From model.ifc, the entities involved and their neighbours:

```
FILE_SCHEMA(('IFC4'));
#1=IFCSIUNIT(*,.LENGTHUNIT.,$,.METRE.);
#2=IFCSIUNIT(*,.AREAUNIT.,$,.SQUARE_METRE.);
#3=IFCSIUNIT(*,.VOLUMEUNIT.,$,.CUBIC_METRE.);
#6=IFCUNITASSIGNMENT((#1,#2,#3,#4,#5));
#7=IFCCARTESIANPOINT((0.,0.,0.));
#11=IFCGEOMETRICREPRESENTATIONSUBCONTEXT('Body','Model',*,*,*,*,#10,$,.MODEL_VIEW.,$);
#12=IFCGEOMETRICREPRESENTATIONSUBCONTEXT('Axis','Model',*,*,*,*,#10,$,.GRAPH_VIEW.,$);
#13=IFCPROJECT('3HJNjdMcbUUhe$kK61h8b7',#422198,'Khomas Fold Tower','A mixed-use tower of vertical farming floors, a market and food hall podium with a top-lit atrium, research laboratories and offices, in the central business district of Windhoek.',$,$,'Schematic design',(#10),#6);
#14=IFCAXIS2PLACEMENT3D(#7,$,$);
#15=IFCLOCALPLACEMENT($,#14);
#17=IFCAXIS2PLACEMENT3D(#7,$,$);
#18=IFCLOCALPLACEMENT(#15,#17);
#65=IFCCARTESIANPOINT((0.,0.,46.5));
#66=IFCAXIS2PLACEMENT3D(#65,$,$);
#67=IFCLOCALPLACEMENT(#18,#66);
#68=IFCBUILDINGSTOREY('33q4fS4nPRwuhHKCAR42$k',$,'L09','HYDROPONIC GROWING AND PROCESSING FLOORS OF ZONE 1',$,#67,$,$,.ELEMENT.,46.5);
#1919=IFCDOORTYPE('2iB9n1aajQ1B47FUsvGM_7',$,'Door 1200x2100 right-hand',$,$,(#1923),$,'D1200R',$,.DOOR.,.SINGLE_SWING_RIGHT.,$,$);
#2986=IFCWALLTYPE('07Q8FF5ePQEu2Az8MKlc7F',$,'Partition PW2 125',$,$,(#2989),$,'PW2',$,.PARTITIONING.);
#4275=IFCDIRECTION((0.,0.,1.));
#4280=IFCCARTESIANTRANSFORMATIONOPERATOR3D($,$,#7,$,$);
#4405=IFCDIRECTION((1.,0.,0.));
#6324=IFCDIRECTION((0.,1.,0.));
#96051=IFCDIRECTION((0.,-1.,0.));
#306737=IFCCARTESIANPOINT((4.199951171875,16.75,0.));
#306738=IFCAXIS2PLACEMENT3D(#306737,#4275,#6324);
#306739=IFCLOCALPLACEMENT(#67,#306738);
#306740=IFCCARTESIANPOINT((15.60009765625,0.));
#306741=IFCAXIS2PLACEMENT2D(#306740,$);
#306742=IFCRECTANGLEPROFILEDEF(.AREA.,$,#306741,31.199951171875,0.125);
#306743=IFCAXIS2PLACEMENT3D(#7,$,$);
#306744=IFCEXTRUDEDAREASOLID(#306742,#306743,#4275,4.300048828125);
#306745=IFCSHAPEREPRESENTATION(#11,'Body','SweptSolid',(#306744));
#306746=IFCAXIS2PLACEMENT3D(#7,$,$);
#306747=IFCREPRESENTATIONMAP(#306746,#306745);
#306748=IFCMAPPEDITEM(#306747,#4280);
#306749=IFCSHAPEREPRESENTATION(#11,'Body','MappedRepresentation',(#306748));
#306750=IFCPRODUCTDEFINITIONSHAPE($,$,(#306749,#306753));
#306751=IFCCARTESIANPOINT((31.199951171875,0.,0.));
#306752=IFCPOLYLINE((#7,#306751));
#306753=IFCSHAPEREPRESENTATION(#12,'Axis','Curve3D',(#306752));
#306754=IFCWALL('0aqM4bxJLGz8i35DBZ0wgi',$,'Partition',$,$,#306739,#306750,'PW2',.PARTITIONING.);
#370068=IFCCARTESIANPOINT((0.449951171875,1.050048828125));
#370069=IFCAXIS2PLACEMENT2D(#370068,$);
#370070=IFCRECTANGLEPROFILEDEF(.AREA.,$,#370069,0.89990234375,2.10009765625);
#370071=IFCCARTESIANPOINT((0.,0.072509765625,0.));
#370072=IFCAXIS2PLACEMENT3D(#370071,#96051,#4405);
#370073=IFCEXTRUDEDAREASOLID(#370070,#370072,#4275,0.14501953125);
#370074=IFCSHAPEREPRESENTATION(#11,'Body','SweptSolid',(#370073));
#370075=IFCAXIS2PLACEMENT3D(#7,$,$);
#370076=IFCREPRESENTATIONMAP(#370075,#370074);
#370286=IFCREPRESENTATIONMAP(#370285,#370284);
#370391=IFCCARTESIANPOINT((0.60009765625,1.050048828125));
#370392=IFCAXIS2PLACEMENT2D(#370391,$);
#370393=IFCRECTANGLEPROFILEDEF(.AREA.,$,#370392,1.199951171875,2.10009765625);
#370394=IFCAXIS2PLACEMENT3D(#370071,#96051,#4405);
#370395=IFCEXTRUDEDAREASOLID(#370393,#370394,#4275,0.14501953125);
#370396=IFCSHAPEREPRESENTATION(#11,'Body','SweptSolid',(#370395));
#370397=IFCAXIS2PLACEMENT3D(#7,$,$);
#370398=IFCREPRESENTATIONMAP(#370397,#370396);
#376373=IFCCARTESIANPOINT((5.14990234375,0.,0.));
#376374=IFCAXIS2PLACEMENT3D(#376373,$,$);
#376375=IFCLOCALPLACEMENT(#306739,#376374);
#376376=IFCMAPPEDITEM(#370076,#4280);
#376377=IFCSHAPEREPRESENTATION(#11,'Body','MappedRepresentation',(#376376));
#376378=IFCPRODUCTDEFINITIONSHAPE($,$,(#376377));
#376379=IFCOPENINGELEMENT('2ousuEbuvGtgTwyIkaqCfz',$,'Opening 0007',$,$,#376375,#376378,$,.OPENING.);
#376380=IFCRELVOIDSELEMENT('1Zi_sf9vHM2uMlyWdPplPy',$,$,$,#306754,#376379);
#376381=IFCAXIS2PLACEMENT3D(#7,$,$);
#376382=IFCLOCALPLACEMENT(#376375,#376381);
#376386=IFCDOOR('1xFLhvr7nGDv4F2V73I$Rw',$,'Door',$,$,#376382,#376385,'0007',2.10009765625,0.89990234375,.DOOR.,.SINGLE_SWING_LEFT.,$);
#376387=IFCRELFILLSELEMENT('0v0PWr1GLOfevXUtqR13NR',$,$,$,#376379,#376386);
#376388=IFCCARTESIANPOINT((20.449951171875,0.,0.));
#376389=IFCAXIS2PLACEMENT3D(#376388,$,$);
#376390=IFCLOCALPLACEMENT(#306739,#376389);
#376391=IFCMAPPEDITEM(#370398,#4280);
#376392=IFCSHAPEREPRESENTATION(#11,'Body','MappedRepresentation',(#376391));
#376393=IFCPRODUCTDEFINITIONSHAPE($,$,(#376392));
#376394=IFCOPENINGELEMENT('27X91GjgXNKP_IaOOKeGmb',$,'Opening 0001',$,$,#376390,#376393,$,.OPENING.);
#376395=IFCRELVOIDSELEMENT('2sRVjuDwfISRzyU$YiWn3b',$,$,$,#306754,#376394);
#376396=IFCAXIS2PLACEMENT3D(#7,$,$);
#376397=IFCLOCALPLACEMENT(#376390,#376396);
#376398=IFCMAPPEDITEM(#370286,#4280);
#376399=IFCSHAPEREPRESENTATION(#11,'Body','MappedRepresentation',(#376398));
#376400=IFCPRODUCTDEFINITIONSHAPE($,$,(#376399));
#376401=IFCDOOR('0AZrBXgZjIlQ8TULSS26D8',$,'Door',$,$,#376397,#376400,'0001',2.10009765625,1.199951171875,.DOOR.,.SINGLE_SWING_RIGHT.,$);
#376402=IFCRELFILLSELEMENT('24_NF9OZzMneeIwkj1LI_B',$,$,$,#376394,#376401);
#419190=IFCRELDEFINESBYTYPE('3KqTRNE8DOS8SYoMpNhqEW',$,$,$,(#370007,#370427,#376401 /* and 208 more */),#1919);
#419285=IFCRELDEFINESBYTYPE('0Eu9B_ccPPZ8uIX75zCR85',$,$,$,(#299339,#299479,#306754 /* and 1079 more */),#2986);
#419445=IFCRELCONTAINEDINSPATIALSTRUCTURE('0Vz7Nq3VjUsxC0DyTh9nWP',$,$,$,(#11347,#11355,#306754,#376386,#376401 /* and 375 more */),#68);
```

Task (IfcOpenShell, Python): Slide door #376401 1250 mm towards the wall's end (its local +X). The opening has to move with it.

```python
import ifcopenshell
import ifcopenshell.api.geometry
import ifcopenshell.util.placement
import ifcopenshell.util.unit

model = ifcopenshell.open("model.ifc")
unit_scale = ifcopenshell.util.unit.calculate_unit_scale(model)

door = model.by_guid("0AZrBXgZjIlQ8TULSS26D8")
opening = door.FillsVoids[0].RelatingOpeningElement
wall = opening.VoidsElements[0].RelatingBuildingElement

wall_matrix = ifcopenshell.util.placement.get_local_placement(wall.ObjectPlacement)
shift = wall_matrix[:3, 0] * 1.25 / unit_scale
before = ifcopenshell.util.placement.get_local_placement(door.ObjectPlacement)[:3, 3].copy()

# The door is placed relative to its opening, so it follows when the opening moves.
matrix = ifcopenshell.util.placement.get_local_placement(opening.ObjectPlacement)
matrix[:3, 3] += shift
ifcopenshell.api.geometry.edit_object_placement(
    model, product=opening, matrix=matrix, is_si=False, should_transform_children=True
)

after = ifcopenshell.util.placement.get_local_placement(door.ObjectPlacement)[:3, 3]
print("door moved by", (after - before).round(3) + 0.0)

model.write("model_rev.ifc")
```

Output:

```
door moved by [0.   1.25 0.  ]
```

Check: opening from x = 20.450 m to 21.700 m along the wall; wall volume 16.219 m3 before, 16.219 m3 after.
